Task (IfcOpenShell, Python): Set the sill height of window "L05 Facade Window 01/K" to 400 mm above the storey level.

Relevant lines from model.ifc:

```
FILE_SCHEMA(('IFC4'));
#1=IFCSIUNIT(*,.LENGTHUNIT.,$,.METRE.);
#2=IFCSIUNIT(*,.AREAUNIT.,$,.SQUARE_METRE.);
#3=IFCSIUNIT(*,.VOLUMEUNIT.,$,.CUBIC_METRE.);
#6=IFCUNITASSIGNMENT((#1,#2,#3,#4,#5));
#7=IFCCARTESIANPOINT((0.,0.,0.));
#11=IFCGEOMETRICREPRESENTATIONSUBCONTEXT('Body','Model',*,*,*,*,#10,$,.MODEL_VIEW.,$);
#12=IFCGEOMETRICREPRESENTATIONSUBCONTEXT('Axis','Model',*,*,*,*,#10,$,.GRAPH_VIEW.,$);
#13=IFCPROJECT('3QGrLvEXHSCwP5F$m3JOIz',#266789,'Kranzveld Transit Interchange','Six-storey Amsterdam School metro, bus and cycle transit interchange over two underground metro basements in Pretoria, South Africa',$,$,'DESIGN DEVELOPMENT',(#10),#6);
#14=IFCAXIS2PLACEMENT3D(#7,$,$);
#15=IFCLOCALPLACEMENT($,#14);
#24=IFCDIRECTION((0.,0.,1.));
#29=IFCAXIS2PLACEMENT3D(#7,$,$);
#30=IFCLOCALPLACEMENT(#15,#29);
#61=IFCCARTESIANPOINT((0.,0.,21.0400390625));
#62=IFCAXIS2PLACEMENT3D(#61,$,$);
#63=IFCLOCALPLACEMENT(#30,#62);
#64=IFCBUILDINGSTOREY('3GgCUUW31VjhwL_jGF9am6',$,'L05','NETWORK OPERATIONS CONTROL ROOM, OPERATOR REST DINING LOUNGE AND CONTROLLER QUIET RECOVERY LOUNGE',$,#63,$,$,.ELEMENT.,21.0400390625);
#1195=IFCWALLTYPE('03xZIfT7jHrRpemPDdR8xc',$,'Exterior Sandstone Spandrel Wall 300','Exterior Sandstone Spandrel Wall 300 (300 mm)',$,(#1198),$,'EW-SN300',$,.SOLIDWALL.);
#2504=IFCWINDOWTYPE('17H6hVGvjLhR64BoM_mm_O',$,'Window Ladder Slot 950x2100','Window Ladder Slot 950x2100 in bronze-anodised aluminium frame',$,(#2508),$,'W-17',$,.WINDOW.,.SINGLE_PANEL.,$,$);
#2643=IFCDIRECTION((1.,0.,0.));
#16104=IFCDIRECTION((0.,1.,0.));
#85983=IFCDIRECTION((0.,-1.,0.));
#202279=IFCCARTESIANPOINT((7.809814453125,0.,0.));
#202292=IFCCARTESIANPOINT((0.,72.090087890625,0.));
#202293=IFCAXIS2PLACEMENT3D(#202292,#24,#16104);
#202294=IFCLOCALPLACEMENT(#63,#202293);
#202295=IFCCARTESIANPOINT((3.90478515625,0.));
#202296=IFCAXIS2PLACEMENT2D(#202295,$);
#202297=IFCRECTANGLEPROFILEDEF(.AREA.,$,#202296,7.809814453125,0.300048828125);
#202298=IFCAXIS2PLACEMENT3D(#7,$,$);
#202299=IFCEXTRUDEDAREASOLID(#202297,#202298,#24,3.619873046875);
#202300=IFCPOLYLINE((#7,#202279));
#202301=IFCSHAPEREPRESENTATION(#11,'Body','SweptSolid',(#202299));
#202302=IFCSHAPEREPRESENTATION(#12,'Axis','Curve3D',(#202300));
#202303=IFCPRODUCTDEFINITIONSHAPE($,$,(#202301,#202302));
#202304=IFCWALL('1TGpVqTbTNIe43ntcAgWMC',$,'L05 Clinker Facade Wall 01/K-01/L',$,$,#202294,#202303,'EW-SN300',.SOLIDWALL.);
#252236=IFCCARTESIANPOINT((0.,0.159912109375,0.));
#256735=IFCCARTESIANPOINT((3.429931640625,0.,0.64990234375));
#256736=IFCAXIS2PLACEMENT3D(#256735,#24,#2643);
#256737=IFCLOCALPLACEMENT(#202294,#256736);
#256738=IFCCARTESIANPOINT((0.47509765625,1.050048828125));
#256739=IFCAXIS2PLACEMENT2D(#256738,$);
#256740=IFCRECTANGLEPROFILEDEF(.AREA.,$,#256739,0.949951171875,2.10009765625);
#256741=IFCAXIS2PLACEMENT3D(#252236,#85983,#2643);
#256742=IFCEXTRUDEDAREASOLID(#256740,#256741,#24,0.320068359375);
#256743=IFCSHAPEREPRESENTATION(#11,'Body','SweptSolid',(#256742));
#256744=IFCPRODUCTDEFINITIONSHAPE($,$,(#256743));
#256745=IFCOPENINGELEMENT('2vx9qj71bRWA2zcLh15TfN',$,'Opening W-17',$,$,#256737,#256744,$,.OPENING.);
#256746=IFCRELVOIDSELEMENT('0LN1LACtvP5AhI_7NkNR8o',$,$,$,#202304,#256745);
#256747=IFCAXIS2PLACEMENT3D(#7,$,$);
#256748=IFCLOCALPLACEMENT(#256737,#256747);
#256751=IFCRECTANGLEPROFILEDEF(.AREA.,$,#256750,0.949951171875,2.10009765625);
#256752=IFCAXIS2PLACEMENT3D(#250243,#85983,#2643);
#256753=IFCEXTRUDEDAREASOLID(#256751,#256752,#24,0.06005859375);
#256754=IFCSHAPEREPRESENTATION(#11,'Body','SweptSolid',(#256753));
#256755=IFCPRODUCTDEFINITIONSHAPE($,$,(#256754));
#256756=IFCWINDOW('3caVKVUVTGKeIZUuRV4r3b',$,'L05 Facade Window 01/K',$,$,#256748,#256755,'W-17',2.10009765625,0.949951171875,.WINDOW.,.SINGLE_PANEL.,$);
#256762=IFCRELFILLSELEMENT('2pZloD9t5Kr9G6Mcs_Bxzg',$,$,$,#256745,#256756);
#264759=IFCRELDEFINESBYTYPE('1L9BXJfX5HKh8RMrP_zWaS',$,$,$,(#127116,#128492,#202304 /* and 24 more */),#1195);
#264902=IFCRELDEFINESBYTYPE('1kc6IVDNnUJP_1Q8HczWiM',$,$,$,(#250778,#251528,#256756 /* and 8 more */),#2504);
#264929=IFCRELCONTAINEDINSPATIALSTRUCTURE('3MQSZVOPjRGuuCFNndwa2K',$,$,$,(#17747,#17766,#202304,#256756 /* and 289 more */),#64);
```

```python
import numpy as np
import ifcopenshell
import ifcopenshell.api.geometry
import ifcopenshell.geom
import ifcopenshell.util.element
import ifcopenshell.util.placement
import ifcopenshell.util.shape
import ifcopenshell.util.unit

model = ifcopenshell.open("model.ifc")
unit_scale = ifcopenshell.util.unit.calculate_unit_scale(model)

window = model.by_guid("3caVKVUVTGKeIZUuRV4r3b")
opening = window.FillsVoids[0].RelatingOpeningElement
storey = ifcopenshell.util.element.get_container(window, ifc_class="IfcBuildingStorey")
level = ifcopenshell.util.placement.get_local_placement(storey.ObjectPlacement)[2, 3]

# The opening's origin need not be at the sill, so measure its lowest point.
shape = ifcopenshell.geom.create_shape(ifcopenshell.geom.settings(), opening)
bottom = ifcopenshell.util.shape.get_shape_bottom_elevation(shape, shape.geometry) / unit_scale
dz = level + 0.4 / unit_scale - bottom

shift = np.array([0.0, 0.0, dz])
# The window is placed relative to its opening, so it follows when the opening moves.
matrix = ifcopenshell.util.placement.get_local_placement(opening.ObjectPlacement)
matrix[:3, 3] += shift
ifcopenshell.api.geometry.edit_object_placement(
    model, product=opening, matrix=matrix, is_si=False, should_transform_children=True
)

print(f"moved by {dz * unit_scale:+.3f} m")

model.write("model_rev.ifc")
```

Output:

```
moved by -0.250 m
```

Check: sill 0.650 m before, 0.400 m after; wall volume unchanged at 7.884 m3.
